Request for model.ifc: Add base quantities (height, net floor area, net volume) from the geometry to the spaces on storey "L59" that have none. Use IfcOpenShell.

First a look at what the model holds.

```python
import ifcopenshell
import ifcopenshell.util.element
import ifcopenshell.util.unit

model = ifcopenshell.open("model.ifc")
print(model.schema)
for unit_type in ("LENGTHUNIT", "AREAUNIT", "VOLUMEUNIT"):
    print(unit_type, ifcopenshell.util.unit.calculate_unit_scale(model, unit_type))
storey = next(s for s in model.by_type("IfcBuildingStorey") if s.Name == "L59")
spaces = [e for e in ifcopenshell.util.element.get_decomposition(storey) if e.is_a("IfcSpace")]
for e in sorted(spaces, key=lambda e: e.id()):
    print(e.id(), e.is_a(), e.Name, list(ifcopenshell.util.element.get_psets(e, qtos_only=True)), sep=" | ")
```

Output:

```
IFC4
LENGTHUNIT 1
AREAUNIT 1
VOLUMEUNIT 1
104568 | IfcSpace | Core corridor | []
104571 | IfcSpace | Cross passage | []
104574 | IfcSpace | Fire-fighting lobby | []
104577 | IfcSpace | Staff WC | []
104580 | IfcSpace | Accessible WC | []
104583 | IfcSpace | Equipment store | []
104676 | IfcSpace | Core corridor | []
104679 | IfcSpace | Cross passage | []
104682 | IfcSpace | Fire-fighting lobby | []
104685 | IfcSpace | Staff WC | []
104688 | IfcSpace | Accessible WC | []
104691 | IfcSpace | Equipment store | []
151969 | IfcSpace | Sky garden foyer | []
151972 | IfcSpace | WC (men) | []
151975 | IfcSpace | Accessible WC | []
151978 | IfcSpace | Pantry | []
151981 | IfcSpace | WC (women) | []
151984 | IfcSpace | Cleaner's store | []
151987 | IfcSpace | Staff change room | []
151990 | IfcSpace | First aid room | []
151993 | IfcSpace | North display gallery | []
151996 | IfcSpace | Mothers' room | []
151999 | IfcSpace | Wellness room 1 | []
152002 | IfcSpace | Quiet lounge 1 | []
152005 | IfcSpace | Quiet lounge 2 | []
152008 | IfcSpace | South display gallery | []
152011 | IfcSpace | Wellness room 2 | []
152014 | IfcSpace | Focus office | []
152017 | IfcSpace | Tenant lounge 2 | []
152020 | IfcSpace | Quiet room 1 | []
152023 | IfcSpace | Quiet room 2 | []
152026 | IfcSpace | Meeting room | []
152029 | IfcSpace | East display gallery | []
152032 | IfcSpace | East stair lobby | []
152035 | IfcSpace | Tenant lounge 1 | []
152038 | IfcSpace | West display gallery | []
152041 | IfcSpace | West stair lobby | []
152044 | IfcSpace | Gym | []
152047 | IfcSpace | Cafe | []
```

```python
import ifcopenshell
import ifcopenshell.api.pset
import ifcopenshell.geom
import ifcopenshell.util.element
import ifcopenshell.util.shape
import ifcopenshell.util.unit

model = ifcopenshell.open("model.ifc")
unit_scale = ifcopenshell.util.unit.calculate_unit_scale(model)
area_scale = ifcopenshell.util.unit.calculate_unit_scale(model, "AREAUNIT")
volume_scale = ifcopenshell.util.unit.calculate_unit_scale(model, "VOLUMEUNIT")
settings = ifcopenshell.geom.settings()

storey = next(s for s in model.by_type("IfcBuildingStorey") if s.Name == "L59")
spaces = [e for e in ifcopenshell.util.element.get_decomposition(storey) if e.is_a("IfcSpace")]

for e in sorted(spaces, key=lambda e: e.id()):
    if ifcopenshell.util.element.get_psets(e, qtos_only=True, should_inherit=False):
        continue
    # Geometry comes back in metres, in the element's own axes.
    shape = ifcopenshell.geom.create_shape(settings, e)
    values = {
        "Height": ifcopenshell.util.shape.get_z(shape.geometry) / unit_scale,
        "NetFloorArea": ifcopenshell.util.shape.get_footprint_area(shape.geometry) / area_scale,
        "NetVolume": ifcopenshell.util.shape.get_volume(shape.geometry) / volume_scale,
    }
    qto = ifcopenshell.api.pset.add_qto(model, product=e, name="Qto_SpaceBaseQuantities")
    ifcopenshell.api.pset.edit_qto(model, qto=qto, properties=values)
    print(e.id(), {k: round(v, 3) for k, v in values.items()})

model.write("model_rev.ifc")
```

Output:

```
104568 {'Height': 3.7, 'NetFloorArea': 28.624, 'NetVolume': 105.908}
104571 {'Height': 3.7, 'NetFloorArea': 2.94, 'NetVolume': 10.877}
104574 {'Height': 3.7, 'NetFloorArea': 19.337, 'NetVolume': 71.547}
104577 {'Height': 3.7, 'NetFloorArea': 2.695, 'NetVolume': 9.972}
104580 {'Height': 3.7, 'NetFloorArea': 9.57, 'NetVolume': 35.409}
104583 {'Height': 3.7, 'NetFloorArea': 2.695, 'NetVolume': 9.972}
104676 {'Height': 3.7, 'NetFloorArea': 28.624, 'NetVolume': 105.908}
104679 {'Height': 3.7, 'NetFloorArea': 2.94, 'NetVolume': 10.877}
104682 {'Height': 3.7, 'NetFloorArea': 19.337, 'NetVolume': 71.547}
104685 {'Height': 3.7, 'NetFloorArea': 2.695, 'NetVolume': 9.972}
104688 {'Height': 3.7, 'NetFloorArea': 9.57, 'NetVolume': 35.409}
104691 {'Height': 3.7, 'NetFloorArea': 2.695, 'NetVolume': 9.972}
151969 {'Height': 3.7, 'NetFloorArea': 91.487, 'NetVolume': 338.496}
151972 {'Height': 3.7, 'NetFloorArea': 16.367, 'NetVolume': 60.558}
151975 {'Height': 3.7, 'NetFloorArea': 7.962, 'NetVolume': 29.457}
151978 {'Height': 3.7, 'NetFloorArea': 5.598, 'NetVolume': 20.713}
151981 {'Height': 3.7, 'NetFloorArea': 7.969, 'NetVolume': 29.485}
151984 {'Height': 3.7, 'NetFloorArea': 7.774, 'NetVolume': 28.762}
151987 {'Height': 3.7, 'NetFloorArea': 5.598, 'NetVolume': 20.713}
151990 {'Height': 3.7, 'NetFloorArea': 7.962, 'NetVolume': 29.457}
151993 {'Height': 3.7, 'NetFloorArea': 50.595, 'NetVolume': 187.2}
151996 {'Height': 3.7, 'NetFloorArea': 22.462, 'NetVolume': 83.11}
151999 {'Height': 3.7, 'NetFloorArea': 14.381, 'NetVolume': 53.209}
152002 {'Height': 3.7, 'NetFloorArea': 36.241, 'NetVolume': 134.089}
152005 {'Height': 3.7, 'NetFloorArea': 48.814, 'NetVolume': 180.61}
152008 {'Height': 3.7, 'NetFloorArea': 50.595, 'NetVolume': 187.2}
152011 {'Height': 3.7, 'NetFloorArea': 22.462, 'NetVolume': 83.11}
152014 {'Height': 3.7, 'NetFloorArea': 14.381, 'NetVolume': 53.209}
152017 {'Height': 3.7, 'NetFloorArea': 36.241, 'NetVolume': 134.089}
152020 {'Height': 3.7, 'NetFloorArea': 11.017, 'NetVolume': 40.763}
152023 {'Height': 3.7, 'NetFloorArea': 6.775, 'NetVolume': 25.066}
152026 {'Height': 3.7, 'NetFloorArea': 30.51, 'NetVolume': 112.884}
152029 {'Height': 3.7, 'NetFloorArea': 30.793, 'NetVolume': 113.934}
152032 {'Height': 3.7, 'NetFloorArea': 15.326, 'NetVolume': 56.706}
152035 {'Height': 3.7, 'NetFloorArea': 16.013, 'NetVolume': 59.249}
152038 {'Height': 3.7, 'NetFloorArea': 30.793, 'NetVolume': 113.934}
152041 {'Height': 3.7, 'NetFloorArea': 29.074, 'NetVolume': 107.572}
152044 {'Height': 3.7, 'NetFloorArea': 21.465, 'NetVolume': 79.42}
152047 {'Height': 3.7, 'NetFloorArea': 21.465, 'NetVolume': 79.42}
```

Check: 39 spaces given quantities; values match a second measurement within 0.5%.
